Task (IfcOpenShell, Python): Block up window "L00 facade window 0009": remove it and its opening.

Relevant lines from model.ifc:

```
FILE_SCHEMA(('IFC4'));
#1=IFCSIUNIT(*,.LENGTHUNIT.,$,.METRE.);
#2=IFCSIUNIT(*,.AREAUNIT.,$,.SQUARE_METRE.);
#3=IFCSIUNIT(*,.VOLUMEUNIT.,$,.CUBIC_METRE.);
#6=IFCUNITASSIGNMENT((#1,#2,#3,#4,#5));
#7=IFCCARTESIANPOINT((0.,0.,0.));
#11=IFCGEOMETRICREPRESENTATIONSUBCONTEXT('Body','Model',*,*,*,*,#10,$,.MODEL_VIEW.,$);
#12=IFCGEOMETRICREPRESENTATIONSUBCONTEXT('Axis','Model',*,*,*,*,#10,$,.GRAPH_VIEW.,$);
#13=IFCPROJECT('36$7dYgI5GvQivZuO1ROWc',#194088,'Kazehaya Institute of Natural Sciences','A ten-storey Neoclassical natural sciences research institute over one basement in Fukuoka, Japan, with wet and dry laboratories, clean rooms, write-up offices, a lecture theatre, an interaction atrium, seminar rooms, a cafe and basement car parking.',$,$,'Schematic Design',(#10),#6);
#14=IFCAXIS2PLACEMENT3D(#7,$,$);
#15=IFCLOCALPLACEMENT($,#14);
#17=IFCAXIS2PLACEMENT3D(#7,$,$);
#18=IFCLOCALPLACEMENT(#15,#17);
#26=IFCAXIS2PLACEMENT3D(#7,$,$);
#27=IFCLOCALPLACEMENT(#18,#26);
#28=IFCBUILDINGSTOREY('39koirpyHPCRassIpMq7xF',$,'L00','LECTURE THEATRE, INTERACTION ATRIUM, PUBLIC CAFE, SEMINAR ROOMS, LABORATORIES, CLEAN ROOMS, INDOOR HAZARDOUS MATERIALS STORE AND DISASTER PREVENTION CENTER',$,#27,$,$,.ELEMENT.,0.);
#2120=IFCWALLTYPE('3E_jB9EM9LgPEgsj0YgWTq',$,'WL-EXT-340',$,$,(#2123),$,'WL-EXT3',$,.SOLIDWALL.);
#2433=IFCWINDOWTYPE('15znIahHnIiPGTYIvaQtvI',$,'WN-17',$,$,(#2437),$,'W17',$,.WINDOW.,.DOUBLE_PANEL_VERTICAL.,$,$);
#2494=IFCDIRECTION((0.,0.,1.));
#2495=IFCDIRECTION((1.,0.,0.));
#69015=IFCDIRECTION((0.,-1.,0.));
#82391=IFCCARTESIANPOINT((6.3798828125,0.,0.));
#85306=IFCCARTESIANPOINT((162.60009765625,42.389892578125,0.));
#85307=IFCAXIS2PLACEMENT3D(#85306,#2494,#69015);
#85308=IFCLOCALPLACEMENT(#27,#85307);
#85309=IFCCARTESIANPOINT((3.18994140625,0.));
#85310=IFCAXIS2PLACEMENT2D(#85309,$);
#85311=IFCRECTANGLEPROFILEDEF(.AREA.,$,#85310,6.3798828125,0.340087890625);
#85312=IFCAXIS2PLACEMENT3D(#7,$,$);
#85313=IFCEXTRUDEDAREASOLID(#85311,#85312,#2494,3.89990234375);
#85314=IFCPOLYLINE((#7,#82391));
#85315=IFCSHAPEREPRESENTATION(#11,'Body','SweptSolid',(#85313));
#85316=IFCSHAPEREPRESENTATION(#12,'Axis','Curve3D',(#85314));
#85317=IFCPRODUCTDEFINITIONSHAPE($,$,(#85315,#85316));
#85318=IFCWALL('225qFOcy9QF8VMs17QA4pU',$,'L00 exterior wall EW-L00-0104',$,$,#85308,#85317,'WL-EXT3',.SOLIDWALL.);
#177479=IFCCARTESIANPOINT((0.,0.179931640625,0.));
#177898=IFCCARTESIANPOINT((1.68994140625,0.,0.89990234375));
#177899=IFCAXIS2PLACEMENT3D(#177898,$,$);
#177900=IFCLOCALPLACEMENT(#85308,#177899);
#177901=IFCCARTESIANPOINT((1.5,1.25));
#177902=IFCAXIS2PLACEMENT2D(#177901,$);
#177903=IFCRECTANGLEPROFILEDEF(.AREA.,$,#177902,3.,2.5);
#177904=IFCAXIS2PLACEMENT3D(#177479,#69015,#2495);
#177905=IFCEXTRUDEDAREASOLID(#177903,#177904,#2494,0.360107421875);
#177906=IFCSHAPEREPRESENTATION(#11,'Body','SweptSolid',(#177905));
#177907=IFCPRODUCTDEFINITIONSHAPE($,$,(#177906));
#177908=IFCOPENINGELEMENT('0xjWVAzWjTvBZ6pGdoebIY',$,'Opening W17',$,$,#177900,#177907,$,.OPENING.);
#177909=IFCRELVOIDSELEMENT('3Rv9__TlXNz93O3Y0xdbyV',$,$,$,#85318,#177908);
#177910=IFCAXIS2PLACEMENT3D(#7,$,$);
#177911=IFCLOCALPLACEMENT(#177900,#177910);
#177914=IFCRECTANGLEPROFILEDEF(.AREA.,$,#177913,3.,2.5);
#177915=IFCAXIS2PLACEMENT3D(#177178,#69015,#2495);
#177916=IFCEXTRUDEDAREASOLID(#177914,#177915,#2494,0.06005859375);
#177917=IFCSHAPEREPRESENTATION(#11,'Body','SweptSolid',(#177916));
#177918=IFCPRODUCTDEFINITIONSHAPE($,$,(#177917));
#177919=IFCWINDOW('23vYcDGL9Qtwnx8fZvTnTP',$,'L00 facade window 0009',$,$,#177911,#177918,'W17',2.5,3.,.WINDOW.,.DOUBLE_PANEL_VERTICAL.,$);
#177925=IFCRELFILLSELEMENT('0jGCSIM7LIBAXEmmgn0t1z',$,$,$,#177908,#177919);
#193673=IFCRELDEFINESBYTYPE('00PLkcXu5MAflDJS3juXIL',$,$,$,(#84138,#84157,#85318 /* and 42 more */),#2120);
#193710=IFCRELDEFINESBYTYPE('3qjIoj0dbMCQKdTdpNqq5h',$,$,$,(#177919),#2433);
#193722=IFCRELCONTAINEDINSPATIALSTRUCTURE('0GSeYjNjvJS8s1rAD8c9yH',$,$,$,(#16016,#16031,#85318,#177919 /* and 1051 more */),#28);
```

```python
import ifcopenshell
import ifcopenshell.api.feature
import ifcopenshell.api.root
import ifcopenshell.geom
import ifcopenshell.util.shape

model = ifcopenshell.open("model.ifc")
settings = ifcopenshell.geom.settings()


def volume(element):
    """Net volume in cubic metres, openings subtracted."""
    shape = ifcopenshell.geom.create_shape(settings, element)
    return ifcopenshell.util.shape.get_volume(shape.geometry)


window = model.by_id(177919)
opening = window.FillsVoids[0].RelatingOpeningElement
wall = opening.VoidsElements[0].RelatingBuildingElement
before = volume(wall)

ifcopenshell.api.root.remove_product(model, product=window)
ifcopenshell.api.feature.remove_feature(model, feature=opening)

after = volume(wall)

print(f"wall volume {before:.3f} -> {after:.3f} m3")

model.write("model-out.ifc")
```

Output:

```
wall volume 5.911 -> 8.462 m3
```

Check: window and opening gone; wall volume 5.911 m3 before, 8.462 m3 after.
